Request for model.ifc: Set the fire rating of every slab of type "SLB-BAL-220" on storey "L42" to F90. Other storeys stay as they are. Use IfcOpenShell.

First a look at what the model holds.

```python
import ifcopenshell
import ifcopenshell.util.element

model = ifcopenshell.open("model.ifc")
print(model.schema)
storey = next(s for s in model.by_type("IfcBuildingStorey") if s.Name == "L42")
slabs = [e for e in ifcopenshell.util.element.get_decomposition(storey) if e.is_a("IfcSlab")]
seen = {}
for e in slabs:
    element_type = ifcopenshell.util.element.get_type(e)
    key = (element_type.Name if element_type != e and element_type else None, ifcopenshell.util.element.get_pset(e, "Pset_SlabCommon", "FireRating"))
    seen[key] = seen.get(key, 0) + 1
for (name, value), count in sorted(seen.items(), key=str):
    print(count, "x", name, "|", value)
```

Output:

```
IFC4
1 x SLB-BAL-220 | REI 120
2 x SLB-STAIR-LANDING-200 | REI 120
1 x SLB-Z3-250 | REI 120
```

```python
import ifcopenshell
import ifcopenshell.api.pset
import ifcopenshell.util.element

model = ifcopenshell.open("model.ifc")

storey = next(s for s in model.by_type("IfcBuildingStorey") if s.Name == "L42")
slabs = [e for e in ifcopenshell.util.element.get_decomposition(storey) if e.is_a("IfcSlab")]

count = 0
for e in slabs:
    element_type = ifcopenshell.util.element.get_type(e)
    if element_type in (None, e) or element_type.Name != "SLB-BAL-220":
        continue
    found = ifcopenshell.util.element.get_pset(e, "Pset_SlabCommon", should_inherit=False)
    if found:
        pset = model.by_id(found["id"])
        if len(ifcopenshell.util.element.get_elements_by_pset(pset)) > 1:
            pset = ifcopenshell.api.pset.unshare_pset(model, products=[e], pset=pset)[0]
    else:
        pset = ifcopenshell.api.pset.add_pset(model, product=e, name="Pset_SlabCommon")
    ifcopenshell.api.pset.edit_pset(model, pset=pset, properties={"FireRating": "F90"})
    count += 1

print(count, "slabs updated")

model.write("model_updated.ifc")
```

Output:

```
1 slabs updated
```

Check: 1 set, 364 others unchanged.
